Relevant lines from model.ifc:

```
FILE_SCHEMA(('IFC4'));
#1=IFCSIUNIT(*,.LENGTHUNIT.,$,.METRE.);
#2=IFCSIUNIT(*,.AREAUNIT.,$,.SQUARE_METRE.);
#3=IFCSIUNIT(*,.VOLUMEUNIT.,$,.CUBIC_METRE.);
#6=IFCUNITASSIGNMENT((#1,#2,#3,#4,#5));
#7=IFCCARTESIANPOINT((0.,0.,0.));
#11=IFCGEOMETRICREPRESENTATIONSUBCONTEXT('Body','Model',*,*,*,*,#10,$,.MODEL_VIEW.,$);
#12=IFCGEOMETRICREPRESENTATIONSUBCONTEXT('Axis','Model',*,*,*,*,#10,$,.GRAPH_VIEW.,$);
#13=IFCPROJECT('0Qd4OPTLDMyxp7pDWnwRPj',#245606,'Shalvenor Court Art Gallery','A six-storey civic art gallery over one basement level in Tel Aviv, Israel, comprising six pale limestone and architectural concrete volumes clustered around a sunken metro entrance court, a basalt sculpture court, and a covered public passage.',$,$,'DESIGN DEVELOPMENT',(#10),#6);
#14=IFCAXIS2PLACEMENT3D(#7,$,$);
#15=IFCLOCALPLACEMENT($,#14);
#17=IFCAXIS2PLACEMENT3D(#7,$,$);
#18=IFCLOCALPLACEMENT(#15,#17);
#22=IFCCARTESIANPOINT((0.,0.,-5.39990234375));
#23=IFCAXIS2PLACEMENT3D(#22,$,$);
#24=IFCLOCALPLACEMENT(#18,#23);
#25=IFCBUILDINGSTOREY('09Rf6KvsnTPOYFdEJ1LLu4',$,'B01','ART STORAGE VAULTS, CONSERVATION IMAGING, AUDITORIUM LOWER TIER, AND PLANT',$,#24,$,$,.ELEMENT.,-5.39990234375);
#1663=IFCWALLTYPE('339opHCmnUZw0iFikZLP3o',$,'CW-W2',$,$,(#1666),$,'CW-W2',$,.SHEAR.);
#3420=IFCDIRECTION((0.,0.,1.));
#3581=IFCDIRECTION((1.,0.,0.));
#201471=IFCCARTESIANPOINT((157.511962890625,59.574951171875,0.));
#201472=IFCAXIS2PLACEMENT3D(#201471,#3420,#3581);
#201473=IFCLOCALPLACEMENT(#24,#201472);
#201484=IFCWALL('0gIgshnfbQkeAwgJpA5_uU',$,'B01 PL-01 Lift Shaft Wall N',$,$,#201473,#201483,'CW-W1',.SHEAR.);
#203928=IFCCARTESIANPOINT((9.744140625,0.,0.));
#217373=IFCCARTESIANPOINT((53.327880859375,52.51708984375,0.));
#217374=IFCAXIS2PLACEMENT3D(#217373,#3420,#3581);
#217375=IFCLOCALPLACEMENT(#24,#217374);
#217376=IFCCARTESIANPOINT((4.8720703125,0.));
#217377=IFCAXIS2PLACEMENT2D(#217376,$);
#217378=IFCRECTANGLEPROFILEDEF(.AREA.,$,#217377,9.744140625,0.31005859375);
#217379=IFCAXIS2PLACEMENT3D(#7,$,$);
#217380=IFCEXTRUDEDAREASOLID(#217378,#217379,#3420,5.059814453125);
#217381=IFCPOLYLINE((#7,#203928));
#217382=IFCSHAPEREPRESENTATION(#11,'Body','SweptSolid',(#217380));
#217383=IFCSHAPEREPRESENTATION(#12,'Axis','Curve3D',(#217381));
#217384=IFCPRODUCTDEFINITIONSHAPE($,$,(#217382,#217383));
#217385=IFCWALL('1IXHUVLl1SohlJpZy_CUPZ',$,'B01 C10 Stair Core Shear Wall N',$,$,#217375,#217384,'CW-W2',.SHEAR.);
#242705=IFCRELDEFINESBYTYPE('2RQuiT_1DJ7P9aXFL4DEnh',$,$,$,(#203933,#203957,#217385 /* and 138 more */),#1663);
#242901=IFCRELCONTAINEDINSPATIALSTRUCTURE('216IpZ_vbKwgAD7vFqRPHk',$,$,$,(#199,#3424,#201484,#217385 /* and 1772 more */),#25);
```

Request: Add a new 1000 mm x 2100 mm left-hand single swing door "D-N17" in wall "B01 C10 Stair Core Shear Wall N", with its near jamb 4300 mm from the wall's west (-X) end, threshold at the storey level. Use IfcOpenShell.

```python
import numpy as np
import ifcopenshell
import ifcopenshell.api.feature
import ifcopenshell.api.geometry
import ifcopenshell.api.root
import ifcopenshell.api.spatial
import ifcopenshell.geom
import ifcopenshell.util.element
import ifcopenshell.util.placement
import ifcopenshell.util.representation
import ifcopenshell.util.shape
import ifcopenshell.util.unit

model = ifcopenshell.open("model.ifc")
unit_scale = ifcopenshell.util.unit.calculate_unit_scale(model)
settings = ifcopenshell.geom.settings()


def volume(element):
    """Net volume in cubic metres, openings subtracted."""
    shape = ifcopenshell.geom.create_shape(settings, element)
    return ifcopenshell.util.shape.get_volume(shape.geometry)


wall = model.by_id(217385)
storey = ifcopenshell.util.element.get_container(wall, ifc_class="IfcBuildingStorey")
context = ifcopenshell.util.representation.get_context(model, "Model", "Body", "MODEL_VIEW")
before = volume(wall)

width, height, from_end, sill = 1, 2.1, 4.3, 0.0  # metres

# The wall runs along its own X axis, and the end named is its -X end.
wall_shape = ifcopenshell.geom.create_shape(settings, wall)
x, y, z = ifcopenshell.util.shape.get_vertices(wall_shape.geometry).T
start = x.min() + from_end
face, thickness = float(y.min()), float(y.max() - y.min())
wall_matrix = ifcopenshell.util.placement.get_local_placement(wall.ObjectPlacement)
level = ifcopenshell.util.placement.get_local_placement(storey.ObjectPlacement)[2, 3]


def in_wall(x, y):
    """Placement at x, y metres in the wall's axes, at sill height."""
    matrix = wall_matrix.copy()
    matrix[:, 3] = wall_matrix @ np.array([x / unit_scale, y / unit_scale, 0.0, 1.0])
    matrix[2, 3] = level + sill / unit_scale
    return matrix


# Opening: a box that overshoots both wall faces by 50 mm.
opening = ifcopenshell.api.root.create_entity(model, ifc_class="IfcOpeningElement", predefined_type="OPENING")
box = ifcopenshell.api.geometry.add_wall_representation(
    model, context=context, length=width, height=height, thickness=thickness + 0.1
)
ifcopenshell.api.geometry.assign_representation(model, product=opening, representation=box)
ifcopenshell.api.geometry.edit_object_placement(model, product=opening, matrix=in_wall(start, face - 0.05), is_si=False)
ifcopenshell.api.feature.add_feature(model, feature=opening, element=wall)

door = ifcopenshell.api.root.create_entity(model, ifc_class="IfcDoor", name="D-N17", predefined_type="DOOR")
door.OverallWidth, door.OverallHeight = width / unit_scale, height / unit_scale
door.OperationType = "SINGLE_SWING_LEFT"
body = ifcopenshell.api.geometry.add_door_representation(
    model,
    context=context,
    overall_width=door.OverallWidth,
    overall_height=door.OverallHeight,
    operation_type="SINGLE_SWING_LEFT",
    lining_properties={"LiningDepth": thickness / unit_scale, "ThresholdDepth": thickness / unit_scale},
)
ifcopenshell.api.geometry.assign_representation(model, product=door, representation=body)
ifcopenshell.api.spatial.assign_container(model, products=[door], relating_structure=storey)
ifcopenshell.api.feature.add_filling(model, opening=opening, element=door)

# The lining spans the wall, so the door starts at the wall face.
ifcopenshell.api.geometry.edit_object_placement(model, product=door, matrix=in_wall(start, face), is_si=False)

after = volume(wall)

print(f"wall volume {before:.3f} -> {after:.3f} m3")

model.write("model_edited.ifc")
```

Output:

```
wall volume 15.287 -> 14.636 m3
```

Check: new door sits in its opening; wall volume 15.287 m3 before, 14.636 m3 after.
